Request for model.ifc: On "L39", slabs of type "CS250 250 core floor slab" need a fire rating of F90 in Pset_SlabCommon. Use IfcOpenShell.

First a look at what the model holds.

```python
import ifcopenshell
import ifcopenshell.util.element

model = ifcopenshell.open("model.ifc")
print(model.schema)
storey = next(s for s in model.by_type("IfcBuildingStorey") if s.Name == "L39")
slabs = [e for e in ifcopenshell.util.element.get_decomposition(storey) if e.is_a("IfcSlab")]
seen = {}
for e in slabs:
    element_type = ifcopenshell.util.element.get_type(e)
    key = (element_type.Name if element_type != e and element_type else None, ifcopenshell.util.element.get_pset(e, "Pset_SlabCommon", "FireRating"))
    seen[key] = seen.get(key, 0) + 1
for (name, value), count in sorted(seen.items(), key=str):
    print(count, "x", name, "|", value)
```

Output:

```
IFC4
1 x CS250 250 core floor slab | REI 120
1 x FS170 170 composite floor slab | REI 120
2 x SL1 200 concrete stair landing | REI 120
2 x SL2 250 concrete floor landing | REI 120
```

```python
import ifcopenshell
import ifcopenshell.api.pset
import ifcopenshell.util.element

model = ifcopenshell.open("model.ifc")

storey = next(s for s in model.by_type("IfcBuildingStorey") if s.Name == "L39")
slabs = [e for e in ifcopenshell.util.element.get_decomposition(storey) if e.is_a("IfcSlab")]

count = 0
for e in slabs:
    element_type = ifcopenshell.util.element.get_type(e)
    if element_type in (None, e) or element_type.Name != "CS250 250 core floor slab":
        continue
    # add_pset returns the element's existing set when there is one.
    pset = ifcopenshell.api.pset.add_pset(model, product=e, name="Pset_SlabCommon")
    ifcopenshell.api.pset.edit_pset(model, pset=pset, properties={"FireRating": "F90"})
    count += 1

print(count, "slabs updated")

model.write("model_updated.ifc")
```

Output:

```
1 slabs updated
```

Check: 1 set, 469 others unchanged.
